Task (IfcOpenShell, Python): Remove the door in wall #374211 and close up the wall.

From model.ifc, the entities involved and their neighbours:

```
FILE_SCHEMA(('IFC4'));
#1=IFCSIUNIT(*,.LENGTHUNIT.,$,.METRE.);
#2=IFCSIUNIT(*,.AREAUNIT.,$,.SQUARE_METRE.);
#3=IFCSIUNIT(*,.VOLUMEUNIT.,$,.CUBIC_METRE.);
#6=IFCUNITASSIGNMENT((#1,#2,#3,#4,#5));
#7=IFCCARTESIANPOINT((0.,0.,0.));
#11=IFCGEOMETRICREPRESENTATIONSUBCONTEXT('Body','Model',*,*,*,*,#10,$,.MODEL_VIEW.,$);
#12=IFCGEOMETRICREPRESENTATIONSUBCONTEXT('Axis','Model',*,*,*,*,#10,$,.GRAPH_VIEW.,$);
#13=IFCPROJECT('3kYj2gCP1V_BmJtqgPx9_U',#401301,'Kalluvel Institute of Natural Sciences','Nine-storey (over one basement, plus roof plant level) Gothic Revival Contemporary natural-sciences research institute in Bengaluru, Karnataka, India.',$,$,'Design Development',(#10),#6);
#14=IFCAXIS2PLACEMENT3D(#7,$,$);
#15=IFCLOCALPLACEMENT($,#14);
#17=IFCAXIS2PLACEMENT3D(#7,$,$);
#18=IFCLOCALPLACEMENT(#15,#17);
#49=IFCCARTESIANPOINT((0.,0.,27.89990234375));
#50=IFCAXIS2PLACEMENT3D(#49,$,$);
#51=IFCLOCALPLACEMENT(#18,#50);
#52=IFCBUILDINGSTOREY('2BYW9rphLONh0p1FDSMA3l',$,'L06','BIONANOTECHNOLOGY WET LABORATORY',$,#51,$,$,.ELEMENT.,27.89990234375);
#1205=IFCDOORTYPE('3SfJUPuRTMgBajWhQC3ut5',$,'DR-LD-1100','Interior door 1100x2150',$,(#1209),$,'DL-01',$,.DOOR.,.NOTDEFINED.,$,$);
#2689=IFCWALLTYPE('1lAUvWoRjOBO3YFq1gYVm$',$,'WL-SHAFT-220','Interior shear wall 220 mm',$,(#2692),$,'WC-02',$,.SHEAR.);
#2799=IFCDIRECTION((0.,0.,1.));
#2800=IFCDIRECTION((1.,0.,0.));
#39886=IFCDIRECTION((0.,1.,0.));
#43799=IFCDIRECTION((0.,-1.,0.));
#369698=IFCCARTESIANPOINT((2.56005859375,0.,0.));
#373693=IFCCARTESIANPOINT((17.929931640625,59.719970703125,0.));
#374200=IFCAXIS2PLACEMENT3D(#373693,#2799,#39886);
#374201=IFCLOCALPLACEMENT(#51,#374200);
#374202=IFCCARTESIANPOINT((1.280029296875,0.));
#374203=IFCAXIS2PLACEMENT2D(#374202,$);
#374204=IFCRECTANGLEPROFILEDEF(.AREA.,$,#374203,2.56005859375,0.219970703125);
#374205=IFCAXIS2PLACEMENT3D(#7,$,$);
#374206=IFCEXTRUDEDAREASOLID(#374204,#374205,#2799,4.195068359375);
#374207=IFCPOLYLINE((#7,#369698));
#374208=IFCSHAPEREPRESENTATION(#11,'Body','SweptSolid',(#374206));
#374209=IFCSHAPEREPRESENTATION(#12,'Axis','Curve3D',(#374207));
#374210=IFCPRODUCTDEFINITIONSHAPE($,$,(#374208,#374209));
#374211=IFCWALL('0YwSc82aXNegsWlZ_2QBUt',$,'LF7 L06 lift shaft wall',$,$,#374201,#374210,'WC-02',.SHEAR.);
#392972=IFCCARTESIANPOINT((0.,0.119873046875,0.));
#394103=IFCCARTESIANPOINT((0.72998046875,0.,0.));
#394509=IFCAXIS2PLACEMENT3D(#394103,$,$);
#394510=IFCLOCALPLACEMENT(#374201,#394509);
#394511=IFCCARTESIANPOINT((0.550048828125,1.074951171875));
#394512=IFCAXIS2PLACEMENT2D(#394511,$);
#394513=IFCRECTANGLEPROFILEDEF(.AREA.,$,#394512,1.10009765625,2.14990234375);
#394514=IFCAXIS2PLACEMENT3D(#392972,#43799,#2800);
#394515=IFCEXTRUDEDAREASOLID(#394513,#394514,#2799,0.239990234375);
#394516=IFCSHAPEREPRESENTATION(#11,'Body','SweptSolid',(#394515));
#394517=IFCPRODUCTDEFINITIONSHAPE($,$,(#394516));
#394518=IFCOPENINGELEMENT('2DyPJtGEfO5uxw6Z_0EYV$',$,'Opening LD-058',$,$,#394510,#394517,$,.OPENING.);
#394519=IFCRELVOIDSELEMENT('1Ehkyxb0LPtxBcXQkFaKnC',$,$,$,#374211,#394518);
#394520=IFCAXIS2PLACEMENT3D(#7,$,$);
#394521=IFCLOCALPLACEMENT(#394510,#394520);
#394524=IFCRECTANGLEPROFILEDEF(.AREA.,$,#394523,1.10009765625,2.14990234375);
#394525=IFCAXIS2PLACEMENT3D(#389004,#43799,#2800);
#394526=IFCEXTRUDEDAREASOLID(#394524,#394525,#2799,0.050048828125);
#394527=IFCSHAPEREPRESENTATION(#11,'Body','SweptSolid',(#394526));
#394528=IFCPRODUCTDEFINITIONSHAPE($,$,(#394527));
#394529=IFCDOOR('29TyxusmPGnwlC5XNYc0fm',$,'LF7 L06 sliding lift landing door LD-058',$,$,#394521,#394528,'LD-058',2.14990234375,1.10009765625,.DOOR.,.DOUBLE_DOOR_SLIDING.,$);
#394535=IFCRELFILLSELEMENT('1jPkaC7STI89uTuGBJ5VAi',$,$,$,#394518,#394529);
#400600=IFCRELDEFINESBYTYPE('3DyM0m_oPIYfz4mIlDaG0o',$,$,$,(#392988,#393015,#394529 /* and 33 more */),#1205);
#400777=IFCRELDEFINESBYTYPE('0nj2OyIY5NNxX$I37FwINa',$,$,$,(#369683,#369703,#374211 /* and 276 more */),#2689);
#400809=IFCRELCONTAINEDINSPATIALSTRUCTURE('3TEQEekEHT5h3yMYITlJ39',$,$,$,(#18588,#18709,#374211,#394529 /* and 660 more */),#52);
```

```python
import ifcopenshell
import ifcopenshell.api.feature
import ifcopenshell.api.root
import ifcopenshell.geom
import ifcopenshell.util.shape

model = ifcopenshell.open("model.ifc")
settings = ifcopenshell.geom.settings()


def volume(element):
    """Net volume in cubic metres, openings subtracted."""
    shape = ifcopenshell.geom.create_shape(settings, element)
    return ifcopenshell.util.shape.get_volume(shape.geometry)


door = model.by_guid("29TyxusmPGnwlC5XNYc0fm")
opening = door.FillsVoids[0].RelatingOpeningElement
wall = opening.VoidsElements[0].RelatingBuildingElement
before = volume(wall)

ifcopenshell.api.root.remove_product(model, product=door)
ifcopenshell.api.feature.remove_feature(model, feature=opening)

after = volume(wall)

print(f"wall volume {before:.3f} -> {after:.3f} m3")

model.write("model_updated.ifc")
```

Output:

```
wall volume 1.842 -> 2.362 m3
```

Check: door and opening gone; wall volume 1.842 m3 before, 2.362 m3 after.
